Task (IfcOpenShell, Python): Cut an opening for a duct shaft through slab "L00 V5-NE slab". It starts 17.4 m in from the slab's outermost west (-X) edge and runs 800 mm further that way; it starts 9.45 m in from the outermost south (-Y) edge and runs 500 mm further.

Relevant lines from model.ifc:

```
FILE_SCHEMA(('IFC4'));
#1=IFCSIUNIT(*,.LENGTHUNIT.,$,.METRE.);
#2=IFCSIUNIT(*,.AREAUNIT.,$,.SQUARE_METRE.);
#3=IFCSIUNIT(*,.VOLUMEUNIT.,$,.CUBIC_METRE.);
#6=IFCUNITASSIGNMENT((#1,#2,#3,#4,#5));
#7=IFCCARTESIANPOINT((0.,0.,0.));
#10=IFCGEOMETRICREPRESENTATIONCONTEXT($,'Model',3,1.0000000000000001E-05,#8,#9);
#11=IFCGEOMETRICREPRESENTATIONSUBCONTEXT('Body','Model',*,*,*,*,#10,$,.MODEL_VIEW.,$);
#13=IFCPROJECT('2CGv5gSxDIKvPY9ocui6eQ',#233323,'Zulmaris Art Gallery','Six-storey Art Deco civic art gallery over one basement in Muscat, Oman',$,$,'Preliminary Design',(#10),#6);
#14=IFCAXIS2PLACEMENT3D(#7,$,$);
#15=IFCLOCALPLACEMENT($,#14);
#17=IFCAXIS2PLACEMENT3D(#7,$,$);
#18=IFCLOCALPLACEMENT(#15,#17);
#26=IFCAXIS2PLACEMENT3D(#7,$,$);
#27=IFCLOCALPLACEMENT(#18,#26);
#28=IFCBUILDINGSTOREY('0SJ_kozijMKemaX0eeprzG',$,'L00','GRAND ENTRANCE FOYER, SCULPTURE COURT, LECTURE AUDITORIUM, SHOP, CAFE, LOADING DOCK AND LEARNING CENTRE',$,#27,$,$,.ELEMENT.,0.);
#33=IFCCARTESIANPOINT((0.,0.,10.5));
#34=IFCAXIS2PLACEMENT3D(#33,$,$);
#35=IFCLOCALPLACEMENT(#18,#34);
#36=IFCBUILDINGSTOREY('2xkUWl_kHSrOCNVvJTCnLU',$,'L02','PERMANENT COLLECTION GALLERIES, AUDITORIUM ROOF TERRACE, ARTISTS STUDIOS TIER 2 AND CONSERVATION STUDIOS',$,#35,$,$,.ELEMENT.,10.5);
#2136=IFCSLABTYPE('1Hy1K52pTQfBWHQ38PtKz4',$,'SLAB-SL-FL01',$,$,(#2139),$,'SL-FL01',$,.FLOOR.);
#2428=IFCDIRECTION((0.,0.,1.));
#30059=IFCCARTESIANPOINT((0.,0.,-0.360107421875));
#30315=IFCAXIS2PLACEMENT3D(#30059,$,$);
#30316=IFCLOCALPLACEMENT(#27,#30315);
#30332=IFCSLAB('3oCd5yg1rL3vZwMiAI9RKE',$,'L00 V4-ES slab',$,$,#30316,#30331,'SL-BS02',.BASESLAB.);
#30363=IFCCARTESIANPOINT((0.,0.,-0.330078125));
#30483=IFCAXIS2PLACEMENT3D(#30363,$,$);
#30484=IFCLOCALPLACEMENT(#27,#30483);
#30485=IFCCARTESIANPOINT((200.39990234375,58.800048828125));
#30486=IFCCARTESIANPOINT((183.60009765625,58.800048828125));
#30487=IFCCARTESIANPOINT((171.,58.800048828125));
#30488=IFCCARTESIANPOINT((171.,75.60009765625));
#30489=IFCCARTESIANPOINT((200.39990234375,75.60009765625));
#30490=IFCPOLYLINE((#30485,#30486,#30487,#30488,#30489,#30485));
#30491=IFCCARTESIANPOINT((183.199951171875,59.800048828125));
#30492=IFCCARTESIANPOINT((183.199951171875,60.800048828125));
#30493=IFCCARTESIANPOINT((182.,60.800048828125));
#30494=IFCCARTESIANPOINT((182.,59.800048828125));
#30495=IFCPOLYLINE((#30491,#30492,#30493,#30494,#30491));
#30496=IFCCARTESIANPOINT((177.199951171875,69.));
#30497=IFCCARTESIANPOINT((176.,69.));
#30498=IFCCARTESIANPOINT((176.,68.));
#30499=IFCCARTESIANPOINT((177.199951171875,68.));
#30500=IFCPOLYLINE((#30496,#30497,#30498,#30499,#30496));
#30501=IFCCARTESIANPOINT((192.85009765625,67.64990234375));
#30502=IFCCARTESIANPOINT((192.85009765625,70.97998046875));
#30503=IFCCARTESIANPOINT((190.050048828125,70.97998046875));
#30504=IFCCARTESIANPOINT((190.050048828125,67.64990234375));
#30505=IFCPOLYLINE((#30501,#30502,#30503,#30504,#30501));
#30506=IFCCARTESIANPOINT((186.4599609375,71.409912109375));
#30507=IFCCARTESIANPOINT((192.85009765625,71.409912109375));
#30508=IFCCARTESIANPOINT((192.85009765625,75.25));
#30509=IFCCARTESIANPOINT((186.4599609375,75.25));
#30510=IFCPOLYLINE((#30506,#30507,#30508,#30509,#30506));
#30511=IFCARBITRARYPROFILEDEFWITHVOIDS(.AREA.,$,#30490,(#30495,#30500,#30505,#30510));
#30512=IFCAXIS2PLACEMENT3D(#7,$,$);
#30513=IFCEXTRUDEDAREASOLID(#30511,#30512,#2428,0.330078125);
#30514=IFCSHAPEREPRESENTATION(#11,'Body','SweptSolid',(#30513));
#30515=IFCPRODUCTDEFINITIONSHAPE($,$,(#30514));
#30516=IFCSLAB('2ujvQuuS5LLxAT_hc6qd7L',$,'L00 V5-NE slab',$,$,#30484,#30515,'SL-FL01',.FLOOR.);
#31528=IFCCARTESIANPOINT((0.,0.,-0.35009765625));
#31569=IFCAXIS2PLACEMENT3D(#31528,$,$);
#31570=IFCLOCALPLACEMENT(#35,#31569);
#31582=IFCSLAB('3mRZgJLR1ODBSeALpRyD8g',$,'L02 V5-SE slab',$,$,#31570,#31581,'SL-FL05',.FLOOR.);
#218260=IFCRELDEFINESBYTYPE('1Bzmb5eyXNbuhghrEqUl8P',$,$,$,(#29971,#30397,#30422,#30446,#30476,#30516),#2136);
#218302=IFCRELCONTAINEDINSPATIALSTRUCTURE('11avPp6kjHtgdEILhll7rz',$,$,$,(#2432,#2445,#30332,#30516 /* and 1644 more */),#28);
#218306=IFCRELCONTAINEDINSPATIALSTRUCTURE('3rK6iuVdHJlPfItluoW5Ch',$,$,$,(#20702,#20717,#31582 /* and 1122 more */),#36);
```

```python
import numpy as np
import ifcopenshell
import ifcopenshell.api.feature
import ifcopenshell.api.geometry
import ifcopenshell.api.root
import ifcopenshell.geom
import ifcopenshell.util.placement
import ifcopenshell.util.representation
import ifcopenshell.util.shape
import ifcopenshell.util.unit

model = ifcopenshell.open("model.ifc")
unit_scale = ifcopenshell.util.unit.calculate_unit_scale(model)
settings = ifcopenshell.geom.settings()


def volume(element):
    """Net volume in cubic metres, openings subtracted."""
    shape = ifcopenshell.geom.create_shape(settings, element)
    return ifcopenshell.util.shape.get_volume(shape.geometry)


slab = model.by_id(30516)
before = volume(slab)

# Extent in the slab's own axes, in metres. The edges named are its -X and -Y sides.
slab_shape = ifcopenshell.geom.create_shape(settings, slab)
vertices = ifcopenshell.util.shape.get_vertices(slab_shape.geometry)
x_min, y_min, bottom = vertices.min(axis=0)
top = vertices[:, 2].max()

opening = ifcopenshell.api.root.create_entity(model, ifc_class="IfcOpeningElement", name="Duct shaft opening", predefined_type="OPENING")
context = ifcopenshell.util.representation.get_context(model, "Model", "Body", "MODEL_VIEW")
width, depth = 0.8, 0.5
outline = [(0.0, 0.0), (width, 0.0), (width, depth), (0.0, depth), (0.0, 0.0)]
# Overshoot both faces by 50 mm so the cut is clean.
shape = ifcopenshell.api.geometry.add_slab_representation(
    model, context=context, depth=top - bottom + 0.1, polyline=outline
)
ifcopenshell.api.geometry.assign_representation(model, product=opening, representation=shape)

matrix = ifcopenshell.util.placement.get_local_placement(slab.ObjectPlacement)
matrix[:, 3] = matrix @ np.append(np.array([x_min + 17.4, y_min + 9.45, bottom - 0.05]) / unit_scale, 1.0)
ifcopenshell.api.geometry.edit_object_placement(model, product=opening, matrix=matrix, is_si=False)
ifcopenshell.api.feature.add_feature(model, feature=opening, element=slab)

after = volume(slab)

print(f"slab volume {before:.3f} -> {after:.3f} m3")

model.write("model_v2.ifc")
```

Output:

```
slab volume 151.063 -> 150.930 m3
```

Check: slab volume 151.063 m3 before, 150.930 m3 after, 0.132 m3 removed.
